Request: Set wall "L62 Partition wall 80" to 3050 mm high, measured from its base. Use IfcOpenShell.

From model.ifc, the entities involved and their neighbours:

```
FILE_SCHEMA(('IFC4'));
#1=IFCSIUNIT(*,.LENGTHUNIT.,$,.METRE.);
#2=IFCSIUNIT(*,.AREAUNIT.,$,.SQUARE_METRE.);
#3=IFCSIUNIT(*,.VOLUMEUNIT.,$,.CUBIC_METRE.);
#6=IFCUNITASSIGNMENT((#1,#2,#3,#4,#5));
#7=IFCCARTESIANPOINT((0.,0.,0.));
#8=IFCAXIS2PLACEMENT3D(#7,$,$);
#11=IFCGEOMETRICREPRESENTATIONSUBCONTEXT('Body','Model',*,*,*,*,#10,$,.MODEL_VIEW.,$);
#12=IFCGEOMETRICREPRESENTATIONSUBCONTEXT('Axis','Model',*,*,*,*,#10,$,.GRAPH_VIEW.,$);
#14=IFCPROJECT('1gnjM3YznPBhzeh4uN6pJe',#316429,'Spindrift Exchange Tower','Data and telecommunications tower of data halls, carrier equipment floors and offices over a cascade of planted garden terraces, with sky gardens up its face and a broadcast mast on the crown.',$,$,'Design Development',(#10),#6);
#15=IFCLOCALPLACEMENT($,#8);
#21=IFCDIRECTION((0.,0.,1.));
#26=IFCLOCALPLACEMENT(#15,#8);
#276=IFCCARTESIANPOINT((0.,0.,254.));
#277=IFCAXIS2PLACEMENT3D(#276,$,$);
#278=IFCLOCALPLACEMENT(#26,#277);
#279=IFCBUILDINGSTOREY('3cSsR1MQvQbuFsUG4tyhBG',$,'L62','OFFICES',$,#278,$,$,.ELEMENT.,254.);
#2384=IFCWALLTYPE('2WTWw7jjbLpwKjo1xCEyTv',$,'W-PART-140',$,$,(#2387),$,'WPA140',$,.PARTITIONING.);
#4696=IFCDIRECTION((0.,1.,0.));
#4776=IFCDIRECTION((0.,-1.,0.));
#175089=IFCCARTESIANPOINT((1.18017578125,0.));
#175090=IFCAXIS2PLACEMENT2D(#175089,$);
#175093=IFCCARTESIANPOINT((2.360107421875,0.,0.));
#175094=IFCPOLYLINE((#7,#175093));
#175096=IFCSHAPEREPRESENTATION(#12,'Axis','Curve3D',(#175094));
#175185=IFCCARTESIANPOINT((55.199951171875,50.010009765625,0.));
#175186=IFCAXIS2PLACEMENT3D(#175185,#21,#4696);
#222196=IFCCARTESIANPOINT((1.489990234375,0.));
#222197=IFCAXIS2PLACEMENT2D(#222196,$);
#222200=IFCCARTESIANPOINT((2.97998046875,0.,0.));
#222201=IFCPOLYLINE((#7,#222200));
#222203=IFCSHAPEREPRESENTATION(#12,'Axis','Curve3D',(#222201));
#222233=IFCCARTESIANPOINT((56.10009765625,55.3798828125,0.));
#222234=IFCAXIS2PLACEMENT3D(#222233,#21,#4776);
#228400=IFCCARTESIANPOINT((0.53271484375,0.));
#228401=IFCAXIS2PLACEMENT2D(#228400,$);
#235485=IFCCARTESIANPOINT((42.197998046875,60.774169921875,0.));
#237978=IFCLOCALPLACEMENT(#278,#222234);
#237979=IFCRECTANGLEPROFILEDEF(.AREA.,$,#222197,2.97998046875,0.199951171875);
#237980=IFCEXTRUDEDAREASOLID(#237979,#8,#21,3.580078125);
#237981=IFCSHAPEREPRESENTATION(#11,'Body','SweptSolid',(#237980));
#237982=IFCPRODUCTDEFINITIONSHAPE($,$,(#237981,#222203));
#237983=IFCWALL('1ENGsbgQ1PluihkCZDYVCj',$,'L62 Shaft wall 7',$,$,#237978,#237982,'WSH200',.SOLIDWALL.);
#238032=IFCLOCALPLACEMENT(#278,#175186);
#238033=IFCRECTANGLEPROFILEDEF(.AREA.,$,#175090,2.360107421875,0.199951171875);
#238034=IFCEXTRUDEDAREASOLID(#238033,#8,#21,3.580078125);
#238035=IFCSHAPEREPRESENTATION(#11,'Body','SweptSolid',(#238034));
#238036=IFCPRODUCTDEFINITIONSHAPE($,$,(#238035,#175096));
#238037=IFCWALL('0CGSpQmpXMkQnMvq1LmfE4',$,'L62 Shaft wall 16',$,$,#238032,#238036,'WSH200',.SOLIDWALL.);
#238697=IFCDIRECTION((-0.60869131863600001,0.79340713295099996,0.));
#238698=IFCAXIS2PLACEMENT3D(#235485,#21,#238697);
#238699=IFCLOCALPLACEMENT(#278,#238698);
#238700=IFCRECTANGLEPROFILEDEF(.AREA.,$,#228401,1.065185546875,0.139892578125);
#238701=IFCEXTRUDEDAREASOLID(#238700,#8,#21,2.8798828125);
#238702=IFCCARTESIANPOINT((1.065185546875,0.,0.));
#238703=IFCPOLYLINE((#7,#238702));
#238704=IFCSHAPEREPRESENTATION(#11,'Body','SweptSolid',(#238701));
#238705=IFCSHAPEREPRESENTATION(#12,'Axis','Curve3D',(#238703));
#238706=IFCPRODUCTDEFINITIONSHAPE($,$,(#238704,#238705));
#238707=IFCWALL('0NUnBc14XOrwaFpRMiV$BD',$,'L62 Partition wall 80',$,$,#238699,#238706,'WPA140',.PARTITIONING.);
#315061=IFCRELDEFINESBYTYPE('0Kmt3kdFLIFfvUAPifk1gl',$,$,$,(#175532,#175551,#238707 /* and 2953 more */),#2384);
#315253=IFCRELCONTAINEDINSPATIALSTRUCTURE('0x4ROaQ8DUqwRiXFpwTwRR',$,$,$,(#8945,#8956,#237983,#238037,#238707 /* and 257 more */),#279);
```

```python
import ifcopenshell
import ifcopenshell.geom
import ifcopenshell.util.representation
import ifcopenshell.util.shape

model = ifcopenshell.open("model.ifc")
settings = ifcopenshell.geom.settings()


def volume(element):
    """Net volume in cubic metres, openings subtracted."""
    shape = ifcopenshell.geom.create_shape(settings, element)
    return ifcopenshell.util.shape.get_volume(shape.geometry)


wall = model.by_id(238707)
before = volume(wall)

body = ifcopenshell.util.representation.get_representation(wall, "Model", "Body")
solid = body.Items[0]
old_height = solid.Depth
solid.Depth = 3.05
after = volume(wall)

print(f"height {old_height:g} -> {solid.Depth:g}, volume {before:.3f} -> {after:.3f} m3")

model.write("model_rev.ifc")
```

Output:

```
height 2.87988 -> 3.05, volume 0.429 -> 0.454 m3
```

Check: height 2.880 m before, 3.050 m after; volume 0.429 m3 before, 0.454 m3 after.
